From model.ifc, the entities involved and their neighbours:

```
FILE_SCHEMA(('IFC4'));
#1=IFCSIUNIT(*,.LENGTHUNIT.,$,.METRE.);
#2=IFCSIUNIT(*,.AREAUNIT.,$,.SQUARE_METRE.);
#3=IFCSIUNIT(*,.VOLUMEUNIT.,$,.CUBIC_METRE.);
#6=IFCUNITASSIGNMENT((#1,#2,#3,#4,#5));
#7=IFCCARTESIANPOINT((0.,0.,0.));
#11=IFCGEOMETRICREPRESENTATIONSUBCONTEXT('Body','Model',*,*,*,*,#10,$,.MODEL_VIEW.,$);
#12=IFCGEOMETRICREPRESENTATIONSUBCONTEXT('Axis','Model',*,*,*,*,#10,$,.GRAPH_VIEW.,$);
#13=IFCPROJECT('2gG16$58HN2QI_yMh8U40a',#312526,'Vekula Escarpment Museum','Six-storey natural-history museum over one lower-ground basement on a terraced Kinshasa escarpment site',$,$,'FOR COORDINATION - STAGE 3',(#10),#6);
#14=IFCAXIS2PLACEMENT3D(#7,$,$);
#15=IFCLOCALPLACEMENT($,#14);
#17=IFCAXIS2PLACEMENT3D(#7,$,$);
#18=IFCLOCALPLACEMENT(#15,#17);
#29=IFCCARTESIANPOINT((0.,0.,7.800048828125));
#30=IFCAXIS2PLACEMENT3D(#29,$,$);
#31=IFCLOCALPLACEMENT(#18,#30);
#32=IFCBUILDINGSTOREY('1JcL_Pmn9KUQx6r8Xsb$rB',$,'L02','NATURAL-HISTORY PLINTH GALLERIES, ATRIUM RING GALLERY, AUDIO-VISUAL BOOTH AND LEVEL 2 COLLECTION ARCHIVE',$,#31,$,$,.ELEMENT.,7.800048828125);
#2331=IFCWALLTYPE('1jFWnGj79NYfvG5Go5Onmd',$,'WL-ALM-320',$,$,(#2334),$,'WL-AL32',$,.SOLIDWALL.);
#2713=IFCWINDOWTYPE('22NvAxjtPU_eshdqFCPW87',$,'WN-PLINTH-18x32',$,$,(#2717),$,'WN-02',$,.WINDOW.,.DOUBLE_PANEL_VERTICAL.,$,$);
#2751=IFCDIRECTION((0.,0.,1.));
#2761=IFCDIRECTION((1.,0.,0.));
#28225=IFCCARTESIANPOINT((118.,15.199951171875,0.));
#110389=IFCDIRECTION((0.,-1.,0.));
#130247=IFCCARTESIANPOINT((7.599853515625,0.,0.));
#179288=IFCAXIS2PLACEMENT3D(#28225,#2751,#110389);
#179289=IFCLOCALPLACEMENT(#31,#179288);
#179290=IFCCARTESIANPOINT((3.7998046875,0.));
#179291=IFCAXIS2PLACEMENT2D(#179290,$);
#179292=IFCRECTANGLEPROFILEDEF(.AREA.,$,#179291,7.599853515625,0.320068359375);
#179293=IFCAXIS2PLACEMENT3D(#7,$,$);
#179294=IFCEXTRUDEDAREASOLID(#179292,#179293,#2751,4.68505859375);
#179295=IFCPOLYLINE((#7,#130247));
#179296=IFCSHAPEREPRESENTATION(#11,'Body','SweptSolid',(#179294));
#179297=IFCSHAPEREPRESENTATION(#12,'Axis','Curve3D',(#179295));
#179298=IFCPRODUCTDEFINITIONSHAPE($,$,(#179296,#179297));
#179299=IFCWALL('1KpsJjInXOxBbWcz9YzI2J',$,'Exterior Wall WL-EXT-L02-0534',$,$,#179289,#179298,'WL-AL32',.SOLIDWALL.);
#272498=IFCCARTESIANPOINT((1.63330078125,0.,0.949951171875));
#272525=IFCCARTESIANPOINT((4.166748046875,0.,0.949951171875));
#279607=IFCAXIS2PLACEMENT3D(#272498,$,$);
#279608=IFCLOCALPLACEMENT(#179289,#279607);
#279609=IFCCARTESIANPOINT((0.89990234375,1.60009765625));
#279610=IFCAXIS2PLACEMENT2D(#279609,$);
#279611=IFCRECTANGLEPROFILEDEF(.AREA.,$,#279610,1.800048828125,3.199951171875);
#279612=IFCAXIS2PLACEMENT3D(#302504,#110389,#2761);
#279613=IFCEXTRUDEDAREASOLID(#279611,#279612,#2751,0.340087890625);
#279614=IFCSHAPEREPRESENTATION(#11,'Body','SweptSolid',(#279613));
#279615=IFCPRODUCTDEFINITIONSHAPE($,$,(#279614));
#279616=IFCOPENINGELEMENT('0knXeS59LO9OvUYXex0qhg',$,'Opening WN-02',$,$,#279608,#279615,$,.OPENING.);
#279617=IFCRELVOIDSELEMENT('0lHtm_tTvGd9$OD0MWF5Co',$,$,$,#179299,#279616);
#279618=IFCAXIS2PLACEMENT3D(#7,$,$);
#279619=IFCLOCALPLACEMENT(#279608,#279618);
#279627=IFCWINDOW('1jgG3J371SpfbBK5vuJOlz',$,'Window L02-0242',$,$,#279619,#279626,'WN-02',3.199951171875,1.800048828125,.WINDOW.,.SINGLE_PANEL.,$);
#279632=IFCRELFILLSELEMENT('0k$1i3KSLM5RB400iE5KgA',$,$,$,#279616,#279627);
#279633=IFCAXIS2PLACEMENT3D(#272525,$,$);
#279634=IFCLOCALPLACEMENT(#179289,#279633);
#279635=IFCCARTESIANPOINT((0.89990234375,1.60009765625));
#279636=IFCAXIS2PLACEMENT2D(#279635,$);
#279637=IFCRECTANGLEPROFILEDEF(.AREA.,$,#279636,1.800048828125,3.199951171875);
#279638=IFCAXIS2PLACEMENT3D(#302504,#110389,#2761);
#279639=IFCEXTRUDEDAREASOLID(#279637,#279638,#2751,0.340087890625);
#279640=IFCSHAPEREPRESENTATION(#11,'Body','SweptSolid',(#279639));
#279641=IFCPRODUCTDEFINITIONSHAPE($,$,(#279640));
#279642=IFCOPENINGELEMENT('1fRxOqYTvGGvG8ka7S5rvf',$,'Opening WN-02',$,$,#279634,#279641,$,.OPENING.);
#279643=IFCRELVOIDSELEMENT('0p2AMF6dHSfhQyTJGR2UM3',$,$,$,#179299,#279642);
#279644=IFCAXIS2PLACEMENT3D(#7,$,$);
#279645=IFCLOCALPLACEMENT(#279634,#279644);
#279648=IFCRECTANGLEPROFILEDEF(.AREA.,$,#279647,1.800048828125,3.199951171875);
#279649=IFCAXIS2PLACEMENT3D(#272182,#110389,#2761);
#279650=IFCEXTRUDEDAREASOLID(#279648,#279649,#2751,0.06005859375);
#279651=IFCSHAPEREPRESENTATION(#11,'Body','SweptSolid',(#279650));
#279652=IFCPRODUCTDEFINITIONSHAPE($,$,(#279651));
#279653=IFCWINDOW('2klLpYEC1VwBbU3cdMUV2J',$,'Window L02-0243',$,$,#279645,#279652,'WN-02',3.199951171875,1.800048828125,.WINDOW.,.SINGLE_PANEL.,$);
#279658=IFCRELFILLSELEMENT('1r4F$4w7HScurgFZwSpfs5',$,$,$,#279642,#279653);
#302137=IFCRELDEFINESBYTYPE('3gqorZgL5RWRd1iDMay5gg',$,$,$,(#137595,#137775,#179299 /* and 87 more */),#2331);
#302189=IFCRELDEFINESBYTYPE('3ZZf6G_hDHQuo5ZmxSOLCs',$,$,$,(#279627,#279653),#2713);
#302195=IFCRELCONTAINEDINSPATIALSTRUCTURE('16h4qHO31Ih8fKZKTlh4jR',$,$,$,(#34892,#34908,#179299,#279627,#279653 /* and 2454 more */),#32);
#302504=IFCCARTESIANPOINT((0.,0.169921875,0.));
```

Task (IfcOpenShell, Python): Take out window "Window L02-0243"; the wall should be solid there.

```python
import ifcopenshell
import ifcopenshell.api.feature
import ifcopenshell.api.root
import ifcopenshell.geom
import ifcopenshell.util.shape

model = ifcopenshell.open("model.ifc")
settings = ifcopenshell.geom.settings()


def volume(element):
    """Net volume in cubic metres, openings subtracted."""
    shape = ifcopenshell.geom.create_shape(settings, element)
    return ifcopenshell.util.shape.get_volume(shape.geometry)


window = model.by_id(279653)
opening = window.FillsVoids[0].RelatingOpeningElement
wall = opening.VoidsElements[0].RelatingBuildingElement
before = volume(wall)

ifcopenshell.api.root.remove_product(model, product=window)
ifcopenshell.api.feature.remove_feature(model, feature=opening)

after = volume(wall)

print(f"wall volume {before:.3f} -> {after:.3f} m3")

model.write("model-out.ifc")
```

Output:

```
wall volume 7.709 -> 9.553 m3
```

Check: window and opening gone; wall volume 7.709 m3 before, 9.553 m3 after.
